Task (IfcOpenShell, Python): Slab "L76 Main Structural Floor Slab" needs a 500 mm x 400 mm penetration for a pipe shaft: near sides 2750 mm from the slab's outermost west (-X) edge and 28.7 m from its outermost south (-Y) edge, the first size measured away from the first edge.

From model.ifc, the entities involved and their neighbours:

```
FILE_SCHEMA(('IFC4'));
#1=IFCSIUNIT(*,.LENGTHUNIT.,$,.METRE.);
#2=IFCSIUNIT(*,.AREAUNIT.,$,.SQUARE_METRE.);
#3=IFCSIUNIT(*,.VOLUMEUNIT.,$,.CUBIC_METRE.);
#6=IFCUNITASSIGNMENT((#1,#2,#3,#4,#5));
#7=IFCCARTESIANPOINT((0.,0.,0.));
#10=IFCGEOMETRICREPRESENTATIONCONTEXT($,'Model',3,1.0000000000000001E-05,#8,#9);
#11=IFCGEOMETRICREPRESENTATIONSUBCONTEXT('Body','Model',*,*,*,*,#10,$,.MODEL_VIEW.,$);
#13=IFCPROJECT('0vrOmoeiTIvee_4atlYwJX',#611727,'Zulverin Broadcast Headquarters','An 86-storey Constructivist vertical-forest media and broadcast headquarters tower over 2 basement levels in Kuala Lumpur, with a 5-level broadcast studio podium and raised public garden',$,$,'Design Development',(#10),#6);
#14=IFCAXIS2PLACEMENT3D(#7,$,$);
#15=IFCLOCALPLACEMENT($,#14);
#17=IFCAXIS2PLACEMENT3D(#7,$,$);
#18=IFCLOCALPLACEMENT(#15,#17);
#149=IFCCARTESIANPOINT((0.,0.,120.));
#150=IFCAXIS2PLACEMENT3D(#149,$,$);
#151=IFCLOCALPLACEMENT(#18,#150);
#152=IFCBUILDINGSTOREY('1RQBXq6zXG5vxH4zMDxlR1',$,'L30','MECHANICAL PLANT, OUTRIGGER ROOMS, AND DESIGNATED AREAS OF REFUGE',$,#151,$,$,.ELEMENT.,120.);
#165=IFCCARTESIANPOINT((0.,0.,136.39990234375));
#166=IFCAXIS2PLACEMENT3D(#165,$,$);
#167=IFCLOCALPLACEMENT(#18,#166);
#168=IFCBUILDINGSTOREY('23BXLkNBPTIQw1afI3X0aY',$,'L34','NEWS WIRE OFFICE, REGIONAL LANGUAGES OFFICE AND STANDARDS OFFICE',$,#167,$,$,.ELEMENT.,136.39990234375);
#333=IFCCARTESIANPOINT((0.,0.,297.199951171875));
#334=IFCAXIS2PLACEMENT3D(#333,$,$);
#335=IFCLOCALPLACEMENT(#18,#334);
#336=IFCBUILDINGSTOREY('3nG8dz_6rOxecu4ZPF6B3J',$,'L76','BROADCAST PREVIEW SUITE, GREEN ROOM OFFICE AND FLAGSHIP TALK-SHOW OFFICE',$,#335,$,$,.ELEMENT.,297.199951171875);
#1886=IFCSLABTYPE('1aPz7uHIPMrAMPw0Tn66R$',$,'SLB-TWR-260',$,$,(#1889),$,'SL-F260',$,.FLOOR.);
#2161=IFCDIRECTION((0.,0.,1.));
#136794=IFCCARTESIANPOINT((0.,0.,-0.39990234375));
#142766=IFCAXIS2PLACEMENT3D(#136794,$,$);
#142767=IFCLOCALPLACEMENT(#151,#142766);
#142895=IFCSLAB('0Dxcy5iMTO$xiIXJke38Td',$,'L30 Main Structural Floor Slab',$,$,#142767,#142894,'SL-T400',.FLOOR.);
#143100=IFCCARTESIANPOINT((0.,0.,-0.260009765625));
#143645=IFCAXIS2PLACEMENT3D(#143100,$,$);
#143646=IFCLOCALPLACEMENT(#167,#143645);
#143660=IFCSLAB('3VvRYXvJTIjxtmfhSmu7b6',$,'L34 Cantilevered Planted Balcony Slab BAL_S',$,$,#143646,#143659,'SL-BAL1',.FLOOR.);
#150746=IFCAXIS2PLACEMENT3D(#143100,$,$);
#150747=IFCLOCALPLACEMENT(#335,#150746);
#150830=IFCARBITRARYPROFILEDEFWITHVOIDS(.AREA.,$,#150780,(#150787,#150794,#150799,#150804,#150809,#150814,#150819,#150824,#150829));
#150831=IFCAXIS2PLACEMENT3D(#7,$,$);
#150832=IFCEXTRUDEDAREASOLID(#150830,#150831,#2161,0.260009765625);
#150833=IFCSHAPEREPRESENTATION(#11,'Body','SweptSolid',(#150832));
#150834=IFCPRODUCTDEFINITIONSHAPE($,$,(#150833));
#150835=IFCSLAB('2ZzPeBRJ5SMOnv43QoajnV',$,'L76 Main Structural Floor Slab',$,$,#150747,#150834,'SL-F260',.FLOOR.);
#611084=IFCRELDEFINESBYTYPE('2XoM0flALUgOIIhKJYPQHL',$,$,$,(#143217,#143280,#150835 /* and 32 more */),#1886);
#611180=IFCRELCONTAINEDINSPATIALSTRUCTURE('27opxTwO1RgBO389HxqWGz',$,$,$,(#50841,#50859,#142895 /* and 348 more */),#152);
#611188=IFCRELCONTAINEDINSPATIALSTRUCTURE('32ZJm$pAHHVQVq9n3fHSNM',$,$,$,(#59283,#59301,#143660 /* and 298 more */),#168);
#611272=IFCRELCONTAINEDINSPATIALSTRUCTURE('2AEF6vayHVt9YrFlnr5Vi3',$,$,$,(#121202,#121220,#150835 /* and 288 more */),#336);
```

```python
import numpy as np
import ifcopenshell
import ifcopenshell.api.feature
import ifcopenshell.api.geometry
import ifcopenshell.api.root
import ifcopenshell.geom
import ifcopenshell.util.placement
import ifcopenshell.util.representation
import ifcopenshell.util.shape
import ifcopenshell.util.unit

model = ifcopenshell.open("model.ifc")
unit_scale = ifcopenshell.util.unit.calculate_unit_scale(model)
settings = ifcopenshell.geom.settings()


def volume(element):
    """Net volume in cubic metres, openings subtracted."""
    shape = ifcopenshell.geom.create_shape(settings, element)
    return ifcopenshell.util.shape.get_volume(shape.geometry)


slab = model.by_id(150835)
before = volume(slab)

# Extent in the slab's own axes, in metres. The edges named are its -X and -Y sides.
slab_shape = ifcopenshell.geom.create_shape(settings, slab)
vertices = ifcopenshell.util.shape.get_vertices(slab_shape.geometry)
x_min, y_min, bottom = vertices.min(axis=0)
top = vertices[:, 2].max()

opening = ifcopenshell.api.root.create_entity(model, ifc_class="IfcOpeningElement", name="Pipe shaft opening", predefined_type="OPENING")
context = ifcopenshell.util.representation.get_context(model, "Model", "Body", "MODEL_VIEW")
width, depth = 0.5, 0.4
outline = [(0.0, 0.0), (width, 0.0), (width, depth), (0.0, depth), (0.0, 0.0)]
# Overshoot both faces by 50 mm so the cut is clean.
shape = ifcopenshell.api.geometry.add_slab_representation(
    model, context=context, depth=top - bottom + 0.1, polyline=outline
)
ifcopenshell.api.geometry.assign_representation(model, product=opening, representation=shape)

matrix = ifcopenshell.util.placement.get_local_placement(slab.ObjectPlacement)
matrix[:, 3] = matrix @ np.append(np.array([x_min + 2.75, y_min + 28.7, bottom - 0.05]) / unit_scale, 1.0)
ifcopenshell.api.geometry.edit_object_placement(model, product=opening, matrix=matrix, is_si=False)
ifcopenshell.api.feature.add_feature(model, feature=opening, element=slab)

after = volume(slab)

print(f"slab volume {before:.3f} -> {after:.3f} m3")

model.write("model_rev.ifc")
```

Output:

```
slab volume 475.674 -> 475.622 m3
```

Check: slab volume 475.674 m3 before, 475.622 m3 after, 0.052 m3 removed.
